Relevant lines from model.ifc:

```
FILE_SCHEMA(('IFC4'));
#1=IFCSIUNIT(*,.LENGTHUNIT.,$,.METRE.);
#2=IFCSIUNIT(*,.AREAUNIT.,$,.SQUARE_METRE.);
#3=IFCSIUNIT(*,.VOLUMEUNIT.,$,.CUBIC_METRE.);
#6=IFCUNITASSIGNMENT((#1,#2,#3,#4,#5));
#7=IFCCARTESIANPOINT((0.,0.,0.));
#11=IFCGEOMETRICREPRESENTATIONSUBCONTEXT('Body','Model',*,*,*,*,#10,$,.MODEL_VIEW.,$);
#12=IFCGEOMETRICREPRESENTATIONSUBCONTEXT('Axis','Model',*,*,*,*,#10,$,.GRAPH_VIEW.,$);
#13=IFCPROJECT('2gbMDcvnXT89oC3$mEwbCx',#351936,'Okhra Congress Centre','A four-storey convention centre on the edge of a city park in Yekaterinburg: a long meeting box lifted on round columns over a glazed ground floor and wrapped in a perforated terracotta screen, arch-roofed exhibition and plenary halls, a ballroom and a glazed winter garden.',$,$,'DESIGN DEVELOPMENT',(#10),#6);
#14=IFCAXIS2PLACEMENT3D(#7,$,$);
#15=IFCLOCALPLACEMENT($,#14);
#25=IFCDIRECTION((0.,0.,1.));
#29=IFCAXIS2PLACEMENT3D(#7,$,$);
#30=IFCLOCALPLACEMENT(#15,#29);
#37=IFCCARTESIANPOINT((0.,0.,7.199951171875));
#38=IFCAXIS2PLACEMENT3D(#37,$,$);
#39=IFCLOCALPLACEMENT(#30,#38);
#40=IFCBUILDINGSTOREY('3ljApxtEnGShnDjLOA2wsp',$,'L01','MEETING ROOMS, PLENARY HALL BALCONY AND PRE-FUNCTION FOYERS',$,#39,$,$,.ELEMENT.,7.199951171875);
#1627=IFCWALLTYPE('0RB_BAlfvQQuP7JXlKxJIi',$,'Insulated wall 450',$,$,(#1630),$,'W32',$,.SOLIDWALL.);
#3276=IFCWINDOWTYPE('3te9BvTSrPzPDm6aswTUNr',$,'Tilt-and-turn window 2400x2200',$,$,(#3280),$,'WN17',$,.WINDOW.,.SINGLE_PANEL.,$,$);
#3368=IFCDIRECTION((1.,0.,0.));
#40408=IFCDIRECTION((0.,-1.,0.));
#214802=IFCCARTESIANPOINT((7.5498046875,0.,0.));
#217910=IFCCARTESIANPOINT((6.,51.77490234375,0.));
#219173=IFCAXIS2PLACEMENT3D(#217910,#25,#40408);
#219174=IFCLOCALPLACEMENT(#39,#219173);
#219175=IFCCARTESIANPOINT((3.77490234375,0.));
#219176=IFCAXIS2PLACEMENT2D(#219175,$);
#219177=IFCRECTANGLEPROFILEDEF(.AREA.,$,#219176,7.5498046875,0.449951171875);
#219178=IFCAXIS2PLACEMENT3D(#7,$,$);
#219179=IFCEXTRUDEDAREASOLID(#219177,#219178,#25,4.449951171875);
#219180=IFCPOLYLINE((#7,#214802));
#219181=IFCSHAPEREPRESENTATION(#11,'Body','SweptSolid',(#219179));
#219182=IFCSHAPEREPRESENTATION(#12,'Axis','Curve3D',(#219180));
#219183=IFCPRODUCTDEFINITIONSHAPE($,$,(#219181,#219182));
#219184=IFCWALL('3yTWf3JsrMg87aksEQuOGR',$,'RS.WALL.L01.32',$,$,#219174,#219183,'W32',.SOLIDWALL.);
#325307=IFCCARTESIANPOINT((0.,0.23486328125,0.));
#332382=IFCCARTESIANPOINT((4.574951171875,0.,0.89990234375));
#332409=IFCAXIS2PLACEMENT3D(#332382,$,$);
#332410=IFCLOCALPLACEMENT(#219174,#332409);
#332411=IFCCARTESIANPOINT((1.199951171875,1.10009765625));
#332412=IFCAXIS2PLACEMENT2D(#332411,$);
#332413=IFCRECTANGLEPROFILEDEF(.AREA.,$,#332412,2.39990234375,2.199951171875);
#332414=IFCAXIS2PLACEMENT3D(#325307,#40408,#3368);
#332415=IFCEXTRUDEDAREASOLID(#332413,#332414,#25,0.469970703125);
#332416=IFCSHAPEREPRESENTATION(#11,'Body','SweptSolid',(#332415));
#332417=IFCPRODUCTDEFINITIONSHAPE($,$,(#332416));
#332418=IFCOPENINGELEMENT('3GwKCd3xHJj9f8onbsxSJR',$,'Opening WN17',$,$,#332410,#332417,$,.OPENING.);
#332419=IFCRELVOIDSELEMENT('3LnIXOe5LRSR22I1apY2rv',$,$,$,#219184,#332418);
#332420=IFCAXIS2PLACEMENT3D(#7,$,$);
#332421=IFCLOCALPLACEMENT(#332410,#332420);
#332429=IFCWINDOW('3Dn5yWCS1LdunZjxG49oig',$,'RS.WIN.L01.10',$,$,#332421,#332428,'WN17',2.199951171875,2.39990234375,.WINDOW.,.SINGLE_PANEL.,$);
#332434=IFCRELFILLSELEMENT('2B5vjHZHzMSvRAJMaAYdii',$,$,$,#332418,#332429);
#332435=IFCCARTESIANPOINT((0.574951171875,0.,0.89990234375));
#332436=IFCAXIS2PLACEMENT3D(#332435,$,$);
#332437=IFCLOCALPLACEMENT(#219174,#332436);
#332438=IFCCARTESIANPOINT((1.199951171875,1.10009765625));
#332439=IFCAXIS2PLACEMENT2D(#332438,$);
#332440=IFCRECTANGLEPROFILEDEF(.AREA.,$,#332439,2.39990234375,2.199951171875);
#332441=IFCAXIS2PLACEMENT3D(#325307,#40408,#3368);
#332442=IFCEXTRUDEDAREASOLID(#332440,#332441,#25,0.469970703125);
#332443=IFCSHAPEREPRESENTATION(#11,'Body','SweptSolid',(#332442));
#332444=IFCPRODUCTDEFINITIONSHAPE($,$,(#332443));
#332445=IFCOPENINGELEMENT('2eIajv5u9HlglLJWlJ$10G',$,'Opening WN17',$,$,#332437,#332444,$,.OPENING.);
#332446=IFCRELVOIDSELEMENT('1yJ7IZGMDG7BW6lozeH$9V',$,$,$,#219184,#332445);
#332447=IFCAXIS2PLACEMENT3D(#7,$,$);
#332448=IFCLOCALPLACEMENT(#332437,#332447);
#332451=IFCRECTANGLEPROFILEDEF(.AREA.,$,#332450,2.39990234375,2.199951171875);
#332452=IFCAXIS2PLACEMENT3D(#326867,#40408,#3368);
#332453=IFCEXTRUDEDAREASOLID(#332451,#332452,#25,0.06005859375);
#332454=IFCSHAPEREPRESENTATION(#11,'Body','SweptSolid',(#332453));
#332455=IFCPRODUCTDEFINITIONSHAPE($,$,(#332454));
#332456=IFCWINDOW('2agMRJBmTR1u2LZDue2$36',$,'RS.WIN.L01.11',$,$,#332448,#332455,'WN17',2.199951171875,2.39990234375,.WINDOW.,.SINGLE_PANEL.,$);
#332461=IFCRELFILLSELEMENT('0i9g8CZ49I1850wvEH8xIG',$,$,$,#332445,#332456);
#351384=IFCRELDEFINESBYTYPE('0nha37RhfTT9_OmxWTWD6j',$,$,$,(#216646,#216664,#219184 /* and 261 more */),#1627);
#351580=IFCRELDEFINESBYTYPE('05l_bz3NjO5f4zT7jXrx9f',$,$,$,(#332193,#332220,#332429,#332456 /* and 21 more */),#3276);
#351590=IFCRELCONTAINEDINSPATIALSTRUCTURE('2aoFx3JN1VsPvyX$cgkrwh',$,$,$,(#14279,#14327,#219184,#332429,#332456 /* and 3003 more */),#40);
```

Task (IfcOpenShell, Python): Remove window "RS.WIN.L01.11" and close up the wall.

```python
import ifcopenshell
import ifcopenshell.api.feature
import ifcopenshell.api.root
import ifcopenshell.geom
import ifcopenshell.util.shape

model = ifcopenshell.open("model.ifc")
settings = ifcopenshell.geom.settings()


def volume(element):
    """Net volume in cubic metres, openings subtracted."""
    shape = ifcopenshell.geom.create_shape(settings, element)
    return ifcopenshell.util.shape.get_volume(shape.geometry)


window = model.by_guid("2agMRJBmTR1u2LZDue2$36")
opening = window.FillsVoids[0].RelatingOpeningElement
wall = opening.VoidsElements[0].RelatingBuildingElement
before = volume(wall)

ifcopenshell.api.root.remove_product(model, product=window)
ifcopenshell.api.feature.remove_feature(model, feature=opening)

after = volume(wall)

print(f"wall volume {before:.3f} -> {after:.3f} m3")

model.write("model_v2.ifc")
```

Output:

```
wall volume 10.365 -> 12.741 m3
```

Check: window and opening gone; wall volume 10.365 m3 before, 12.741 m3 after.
